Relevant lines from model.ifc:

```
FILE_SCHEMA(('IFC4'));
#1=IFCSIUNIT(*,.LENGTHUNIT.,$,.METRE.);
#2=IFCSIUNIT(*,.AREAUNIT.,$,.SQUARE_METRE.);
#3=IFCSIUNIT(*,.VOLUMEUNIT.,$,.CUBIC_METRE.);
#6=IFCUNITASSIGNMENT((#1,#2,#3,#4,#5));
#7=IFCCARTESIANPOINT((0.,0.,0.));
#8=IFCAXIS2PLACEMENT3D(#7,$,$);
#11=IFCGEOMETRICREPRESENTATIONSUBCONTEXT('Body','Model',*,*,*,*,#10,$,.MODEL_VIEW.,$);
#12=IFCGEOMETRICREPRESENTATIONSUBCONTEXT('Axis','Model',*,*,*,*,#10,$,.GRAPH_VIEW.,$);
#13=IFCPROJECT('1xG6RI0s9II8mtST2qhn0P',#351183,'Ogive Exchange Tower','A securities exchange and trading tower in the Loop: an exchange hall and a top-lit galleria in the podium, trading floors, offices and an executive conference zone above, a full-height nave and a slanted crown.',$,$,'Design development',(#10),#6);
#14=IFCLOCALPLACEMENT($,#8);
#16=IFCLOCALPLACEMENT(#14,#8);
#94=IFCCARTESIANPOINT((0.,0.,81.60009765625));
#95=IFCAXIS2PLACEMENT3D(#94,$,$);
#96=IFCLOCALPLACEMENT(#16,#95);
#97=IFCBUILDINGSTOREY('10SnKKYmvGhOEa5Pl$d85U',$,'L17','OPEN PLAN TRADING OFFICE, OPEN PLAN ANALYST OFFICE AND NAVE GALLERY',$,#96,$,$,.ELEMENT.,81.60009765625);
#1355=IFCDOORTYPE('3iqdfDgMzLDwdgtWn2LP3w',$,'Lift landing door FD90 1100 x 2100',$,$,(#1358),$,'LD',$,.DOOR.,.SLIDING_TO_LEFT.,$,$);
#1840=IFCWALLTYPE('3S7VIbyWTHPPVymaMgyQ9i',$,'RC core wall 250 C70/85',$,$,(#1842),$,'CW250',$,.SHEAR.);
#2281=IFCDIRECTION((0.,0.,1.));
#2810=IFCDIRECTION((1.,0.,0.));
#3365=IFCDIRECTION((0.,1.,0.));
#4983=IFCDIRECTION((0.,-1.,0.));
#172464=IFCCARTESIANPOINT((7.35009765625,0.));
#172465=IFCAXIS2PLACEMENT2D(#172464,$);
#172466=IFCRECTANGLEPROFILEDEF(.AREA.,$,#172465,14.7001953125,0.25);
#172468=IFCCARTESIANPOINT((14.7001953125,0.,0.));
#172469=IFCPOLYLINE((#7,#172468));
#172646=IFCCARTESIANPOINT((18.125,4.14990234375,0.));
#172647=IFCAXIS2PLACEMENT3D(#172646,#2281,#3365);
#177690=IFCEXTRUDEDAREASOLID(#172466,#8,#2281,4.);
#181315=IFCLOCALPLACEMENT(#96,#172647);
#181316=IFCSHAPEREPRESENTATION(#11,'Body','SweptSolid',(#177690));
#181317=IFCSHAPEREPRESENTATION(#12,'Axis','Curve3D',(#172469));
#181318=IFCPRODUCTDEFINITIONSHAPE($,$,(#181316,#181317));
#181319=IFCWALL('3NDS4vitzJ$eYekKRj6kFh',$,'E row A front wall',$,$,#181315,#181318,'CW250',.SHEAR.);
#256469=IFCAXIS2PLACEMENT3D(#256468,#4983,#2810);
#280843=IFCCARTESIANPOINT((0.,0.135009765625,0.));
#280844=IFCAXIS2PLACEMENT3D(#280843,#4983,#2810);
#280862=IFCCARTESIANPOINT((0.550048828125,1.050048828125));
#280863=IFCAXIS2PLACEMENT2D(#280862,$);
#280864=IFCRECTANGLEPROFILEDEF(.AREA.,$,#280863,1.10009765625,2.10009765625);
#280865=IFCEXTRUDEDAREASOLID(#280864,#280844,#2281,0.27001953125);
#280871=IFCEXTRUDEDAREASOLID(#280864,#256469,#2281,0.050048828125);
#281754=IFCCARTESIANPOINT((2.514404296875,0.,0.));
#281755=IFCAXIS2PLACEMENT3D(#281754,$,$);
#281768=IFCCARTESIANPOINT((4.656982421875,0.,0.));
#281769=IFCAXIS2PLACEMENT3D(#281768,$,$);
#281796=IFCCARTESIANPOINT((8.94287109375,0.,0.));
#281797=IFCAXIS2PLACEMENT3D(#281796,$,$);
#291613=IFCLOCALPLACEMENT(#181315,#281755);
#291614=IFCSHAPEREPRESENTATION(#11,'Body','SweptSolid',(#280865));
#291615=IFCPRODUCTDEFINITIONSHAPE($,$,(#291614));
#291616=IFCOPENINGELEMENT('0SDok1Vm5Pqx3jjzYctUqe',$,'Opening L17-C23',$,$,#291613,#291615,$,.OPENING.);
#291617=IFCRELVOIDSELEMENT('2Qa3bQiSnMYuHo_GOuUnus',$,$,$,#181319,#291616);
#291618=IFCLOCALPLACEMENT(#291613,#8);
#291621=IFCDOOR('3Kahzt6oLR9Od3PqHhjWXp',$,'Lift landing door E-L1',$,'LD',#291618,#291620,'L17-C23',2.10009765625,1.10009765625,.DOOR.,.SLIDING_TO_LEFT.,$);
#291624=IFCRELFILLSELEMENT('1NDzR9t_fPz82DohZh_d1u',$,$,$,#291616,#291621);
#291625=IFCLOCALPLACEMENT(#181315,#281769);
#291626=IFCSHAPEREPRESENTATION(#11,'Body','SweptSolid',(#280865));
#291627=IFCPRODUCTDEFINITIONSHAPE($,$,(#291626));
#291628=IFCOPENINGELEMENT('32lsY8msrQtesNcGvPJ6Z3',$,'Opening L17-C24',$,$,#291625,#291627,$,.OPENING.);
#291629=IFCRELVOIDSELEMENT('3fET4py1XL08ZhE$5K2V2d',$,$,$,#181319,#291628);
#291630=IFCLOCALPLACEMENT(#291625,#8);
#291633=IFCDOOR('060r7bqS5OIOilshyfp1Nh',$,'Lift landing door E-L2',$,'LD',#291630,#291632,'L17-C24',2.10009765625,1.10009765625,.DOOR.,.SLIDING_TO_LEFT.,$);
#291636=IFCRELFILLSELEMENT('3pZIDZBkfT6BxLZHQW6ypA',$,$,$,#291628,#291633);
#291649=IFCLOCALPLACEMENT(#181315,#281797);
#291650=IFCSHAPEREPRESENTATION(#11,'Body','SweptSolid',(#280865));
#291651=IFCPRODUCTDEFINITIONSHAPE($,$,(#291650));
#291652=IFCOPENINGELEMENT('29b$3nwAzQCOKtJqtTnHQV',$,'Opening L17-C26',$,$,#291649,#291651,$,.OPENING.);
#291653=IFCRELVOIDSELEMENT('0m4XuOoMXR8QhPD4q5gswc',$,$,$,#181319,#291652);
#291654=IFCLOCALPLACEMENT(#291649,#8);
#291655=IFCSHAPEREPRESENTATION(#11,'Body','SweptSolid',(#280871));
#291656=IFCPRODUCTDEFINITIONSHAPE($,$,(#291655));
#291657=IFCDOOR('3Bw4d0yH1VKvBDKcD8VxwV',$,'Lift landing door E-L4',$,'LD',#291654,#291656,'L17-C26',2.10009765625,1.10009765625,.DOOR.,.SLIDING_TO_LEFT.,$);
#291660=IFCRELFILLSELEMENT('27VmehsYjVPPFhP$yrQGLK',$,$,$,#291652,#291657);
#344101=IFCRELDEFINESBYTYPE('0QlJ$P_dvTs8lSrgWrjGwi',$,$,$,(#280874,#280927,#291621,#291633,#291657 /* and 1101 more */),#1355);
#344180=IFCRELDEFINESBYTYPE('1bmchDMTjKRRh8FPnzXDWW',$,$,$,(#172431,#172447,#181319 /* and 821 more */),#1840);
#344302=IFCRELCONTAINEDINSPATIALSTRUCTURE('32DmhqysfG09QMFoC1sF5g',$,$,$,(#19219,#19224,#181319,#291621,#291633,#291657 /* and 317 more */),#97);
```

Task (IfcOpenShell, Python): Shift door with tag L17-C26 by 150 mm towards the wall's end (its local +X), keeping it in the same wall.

```python
import ifcopenshell
import ifcopenshell.api.geometry
import ifcopenshell.util.placement
import ifcopenshell.util.unit

model = ifcopenshell.open("model.ifc")
unit_scale = ifcopenshell.util.unit.calculate_unit_scale(model)

door = model.by_guid("3Bw4d0yH1VKvBDKcD8VxwV")
opening = door.FillsVoids[0].RelatingOpeningElement
wall = opening.VoidsElements[0].RelatingBuildingElement

wall_matrix = ifcopenshell.util.placement.get_local_placement(wall.ObjectPlacement)
shift = wall_matrix[:3, 0] * 0.15 / unit_scale
before = ifcopenshell.util.placement.get_local_placement(door.ObjectPlacement)[:3, 3].copy()

# The door is placed relative to its opening, so it follows when the opening moves.
matrix = ifcopenshell.util.placement.get_local_placement(opening.ObjectPlacement)
matrix[:3, 3] += shift
ifcopenshell.api.geometry.edit_object_placement(
    model, product=opening, matrix=matrix, is_si=False, should_transform_children=True
)

after = ifcopenshell.util.placement.get_local_placement(door.ObjectPlacement)[:3, 3]
print("door moved by", (after - before).round(3) + 0.0)

model.write("model_edited.ifc")
```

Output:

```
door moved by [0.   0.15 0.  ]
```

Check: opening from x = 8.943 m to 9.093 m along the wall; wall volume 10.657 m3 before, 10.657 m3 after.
